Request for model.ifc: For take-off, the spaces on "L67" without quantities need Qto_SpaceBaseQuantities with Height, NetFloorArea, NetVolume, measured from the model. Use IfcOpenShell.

First a look at what the model holds.

```python
import ifcopenshell
import ifcopenshell.util.element
import ifcopenshell.util.unit

model = ifcopenshell.open("model.ifc")
print(model.schema)
for unit_type in ("LENGTHUNIT", "AREAUNIT", "VOLUMEUNIT"):
    print(unit_type, ifcopenshell.util.unit.calculate_unit_scale(model, unit_type))
storey = next(s for s in model.by_type("IfcBuildingStorey") if s.Name == "L67")
spaces = [e for e in ifcopenshell.util.element.get_decomposition(storey) if e.is_a("IfcSpace")]
for e in sorted(spaces, key=lambda e: e.id()):
    print(e.id(), e.is_a(), e.Name, list(ifcopenshell.util.element.get_psets(e, qtos_only=True)), sep=" | ")
```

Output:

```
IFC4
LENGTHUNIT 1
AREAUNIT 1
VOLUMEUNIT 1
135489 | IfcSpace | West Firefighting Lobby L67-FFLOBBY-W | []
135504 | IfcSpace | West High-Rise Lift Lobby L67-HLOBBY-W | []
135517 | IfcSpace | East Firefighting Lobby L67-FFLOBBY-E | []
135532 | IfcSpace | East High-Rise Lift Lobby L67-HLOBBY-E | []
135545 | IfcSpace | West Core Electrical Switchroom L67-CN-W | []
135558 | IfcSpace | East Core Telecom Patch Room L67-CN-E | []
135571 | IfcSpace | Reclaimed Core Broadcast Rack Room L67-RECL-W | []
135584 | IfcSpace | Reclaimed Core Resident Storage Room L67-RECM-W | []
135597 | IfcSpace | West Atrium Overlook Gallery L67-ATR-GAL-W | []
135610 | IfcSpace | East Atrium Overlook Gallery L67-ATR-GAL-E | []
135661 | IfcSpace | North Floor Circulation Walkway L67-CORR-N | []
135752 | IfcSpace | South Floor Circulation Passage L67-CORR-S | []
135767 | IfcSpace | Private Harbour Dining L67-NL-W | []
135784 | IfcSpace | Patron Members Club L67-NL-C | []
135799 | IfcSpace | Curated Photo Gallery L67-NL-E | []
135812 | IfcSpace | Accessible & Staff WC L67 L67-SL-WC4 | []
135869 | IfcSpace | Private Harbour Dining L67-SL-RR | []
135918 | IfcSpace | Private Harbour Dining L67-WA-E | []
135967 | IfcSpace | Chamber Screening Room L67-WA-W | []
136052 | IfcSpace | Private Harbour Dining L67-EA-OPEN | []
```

```python
import ifcopenshell
import ifcopenshell.api.pset
import ifcopenshell.geom
import ifcopenshell.util.element
import ifcopenshell.util.shape
import ifcopenshell.util.unit

model = ifcopenshell.open("model.ifc")
unit_scale = ifcopenshell.util.unit.calculate_unit_scale(model)
area_scale = ifcopenshell.util.unit.calculate_unit_scale(model, "AREAUNIT")
volume_scale = ifcopenshell.util.unit.calculate_unit_scale(model, "VOLUMEUNIT")
settings = ifcopenshell.geom.settings()

storey = next(s for s in model.by_type("IfcBuildingStorey") if s.Name == "L67")
spaces = [e for e in ifcopenshell.util.element.get_decomposition(storey) if e.is_a("IfcSpace")]

for e in sorted(spaces, key=lambda e: e.id()):
    if ifcopenshell.util.element.get_psets(e, qtos_only=True, should_inherit=False):
        continue
    # Geometry comes back in metres, in the element's own axes.
    shape = ifcopenshell.geom.create_shape(settings, e)
    values = {
        "Height": ifcopenshell.util.shape.get_z(shape.geometry) / unit_scale,
        "NetFloorArea": ifcopenshell.util.shape.get_footprint_area(shape.geometry) / area_scale,
        "NetVolume": ifcopenshell.util.shape.get_volume(shape.geometry) / volume_scale,
    }
    qto = ifcopenshell.api.pset.add_qto(model, product=e, name="Qto_SpaceBaseQuantities")
    ifcopenshell.api.pset.edit_qto(model, qto=qto, properties=values)
    print(e.id(), {k: round(v, 3) for k, v in values.items()})

model.write("model-out.ifc")
```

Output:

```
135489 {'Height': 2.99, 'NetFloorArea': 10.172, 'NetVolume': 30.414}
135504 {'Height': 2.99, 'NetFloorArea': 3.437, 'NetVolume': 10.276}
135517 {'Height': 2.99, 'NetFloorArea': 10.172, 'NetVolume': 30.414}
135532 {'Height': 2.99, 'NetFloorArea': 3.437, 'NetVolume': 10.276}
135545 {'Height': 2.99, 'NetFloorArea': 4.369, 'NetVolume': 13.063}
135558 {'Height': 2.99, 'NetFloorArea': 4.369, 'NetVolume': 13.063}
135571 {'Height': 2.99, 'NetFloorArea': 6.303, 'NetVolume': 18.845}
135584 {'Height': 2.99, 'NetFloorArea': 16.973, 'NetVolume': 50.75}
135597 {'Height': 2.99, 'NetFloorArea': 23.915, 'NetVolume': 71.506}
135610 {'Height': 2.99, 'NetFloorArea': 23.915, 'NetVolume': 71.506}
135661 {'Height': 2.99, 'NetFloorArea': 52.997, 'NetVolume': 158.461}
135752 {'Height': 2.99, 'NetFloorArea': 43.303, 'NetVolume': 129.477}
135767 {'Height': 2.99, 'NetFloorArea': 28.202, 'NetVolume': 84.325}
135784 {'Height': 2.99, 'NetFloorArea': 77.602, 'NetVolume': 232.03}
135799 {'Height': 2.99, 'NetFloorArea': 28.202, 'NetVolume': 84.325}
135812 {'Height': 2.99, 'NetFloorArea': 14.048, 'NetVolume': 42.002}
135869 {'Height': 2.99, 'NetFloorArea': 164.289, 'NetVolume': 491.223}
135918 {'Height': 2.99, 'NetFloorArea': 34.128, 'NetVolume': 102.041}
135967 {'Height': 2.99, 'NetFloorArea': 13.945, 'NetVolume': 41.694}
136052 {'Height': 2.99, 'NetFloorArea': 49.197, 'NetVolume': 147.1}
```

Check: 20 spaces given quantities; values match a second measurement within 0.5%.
